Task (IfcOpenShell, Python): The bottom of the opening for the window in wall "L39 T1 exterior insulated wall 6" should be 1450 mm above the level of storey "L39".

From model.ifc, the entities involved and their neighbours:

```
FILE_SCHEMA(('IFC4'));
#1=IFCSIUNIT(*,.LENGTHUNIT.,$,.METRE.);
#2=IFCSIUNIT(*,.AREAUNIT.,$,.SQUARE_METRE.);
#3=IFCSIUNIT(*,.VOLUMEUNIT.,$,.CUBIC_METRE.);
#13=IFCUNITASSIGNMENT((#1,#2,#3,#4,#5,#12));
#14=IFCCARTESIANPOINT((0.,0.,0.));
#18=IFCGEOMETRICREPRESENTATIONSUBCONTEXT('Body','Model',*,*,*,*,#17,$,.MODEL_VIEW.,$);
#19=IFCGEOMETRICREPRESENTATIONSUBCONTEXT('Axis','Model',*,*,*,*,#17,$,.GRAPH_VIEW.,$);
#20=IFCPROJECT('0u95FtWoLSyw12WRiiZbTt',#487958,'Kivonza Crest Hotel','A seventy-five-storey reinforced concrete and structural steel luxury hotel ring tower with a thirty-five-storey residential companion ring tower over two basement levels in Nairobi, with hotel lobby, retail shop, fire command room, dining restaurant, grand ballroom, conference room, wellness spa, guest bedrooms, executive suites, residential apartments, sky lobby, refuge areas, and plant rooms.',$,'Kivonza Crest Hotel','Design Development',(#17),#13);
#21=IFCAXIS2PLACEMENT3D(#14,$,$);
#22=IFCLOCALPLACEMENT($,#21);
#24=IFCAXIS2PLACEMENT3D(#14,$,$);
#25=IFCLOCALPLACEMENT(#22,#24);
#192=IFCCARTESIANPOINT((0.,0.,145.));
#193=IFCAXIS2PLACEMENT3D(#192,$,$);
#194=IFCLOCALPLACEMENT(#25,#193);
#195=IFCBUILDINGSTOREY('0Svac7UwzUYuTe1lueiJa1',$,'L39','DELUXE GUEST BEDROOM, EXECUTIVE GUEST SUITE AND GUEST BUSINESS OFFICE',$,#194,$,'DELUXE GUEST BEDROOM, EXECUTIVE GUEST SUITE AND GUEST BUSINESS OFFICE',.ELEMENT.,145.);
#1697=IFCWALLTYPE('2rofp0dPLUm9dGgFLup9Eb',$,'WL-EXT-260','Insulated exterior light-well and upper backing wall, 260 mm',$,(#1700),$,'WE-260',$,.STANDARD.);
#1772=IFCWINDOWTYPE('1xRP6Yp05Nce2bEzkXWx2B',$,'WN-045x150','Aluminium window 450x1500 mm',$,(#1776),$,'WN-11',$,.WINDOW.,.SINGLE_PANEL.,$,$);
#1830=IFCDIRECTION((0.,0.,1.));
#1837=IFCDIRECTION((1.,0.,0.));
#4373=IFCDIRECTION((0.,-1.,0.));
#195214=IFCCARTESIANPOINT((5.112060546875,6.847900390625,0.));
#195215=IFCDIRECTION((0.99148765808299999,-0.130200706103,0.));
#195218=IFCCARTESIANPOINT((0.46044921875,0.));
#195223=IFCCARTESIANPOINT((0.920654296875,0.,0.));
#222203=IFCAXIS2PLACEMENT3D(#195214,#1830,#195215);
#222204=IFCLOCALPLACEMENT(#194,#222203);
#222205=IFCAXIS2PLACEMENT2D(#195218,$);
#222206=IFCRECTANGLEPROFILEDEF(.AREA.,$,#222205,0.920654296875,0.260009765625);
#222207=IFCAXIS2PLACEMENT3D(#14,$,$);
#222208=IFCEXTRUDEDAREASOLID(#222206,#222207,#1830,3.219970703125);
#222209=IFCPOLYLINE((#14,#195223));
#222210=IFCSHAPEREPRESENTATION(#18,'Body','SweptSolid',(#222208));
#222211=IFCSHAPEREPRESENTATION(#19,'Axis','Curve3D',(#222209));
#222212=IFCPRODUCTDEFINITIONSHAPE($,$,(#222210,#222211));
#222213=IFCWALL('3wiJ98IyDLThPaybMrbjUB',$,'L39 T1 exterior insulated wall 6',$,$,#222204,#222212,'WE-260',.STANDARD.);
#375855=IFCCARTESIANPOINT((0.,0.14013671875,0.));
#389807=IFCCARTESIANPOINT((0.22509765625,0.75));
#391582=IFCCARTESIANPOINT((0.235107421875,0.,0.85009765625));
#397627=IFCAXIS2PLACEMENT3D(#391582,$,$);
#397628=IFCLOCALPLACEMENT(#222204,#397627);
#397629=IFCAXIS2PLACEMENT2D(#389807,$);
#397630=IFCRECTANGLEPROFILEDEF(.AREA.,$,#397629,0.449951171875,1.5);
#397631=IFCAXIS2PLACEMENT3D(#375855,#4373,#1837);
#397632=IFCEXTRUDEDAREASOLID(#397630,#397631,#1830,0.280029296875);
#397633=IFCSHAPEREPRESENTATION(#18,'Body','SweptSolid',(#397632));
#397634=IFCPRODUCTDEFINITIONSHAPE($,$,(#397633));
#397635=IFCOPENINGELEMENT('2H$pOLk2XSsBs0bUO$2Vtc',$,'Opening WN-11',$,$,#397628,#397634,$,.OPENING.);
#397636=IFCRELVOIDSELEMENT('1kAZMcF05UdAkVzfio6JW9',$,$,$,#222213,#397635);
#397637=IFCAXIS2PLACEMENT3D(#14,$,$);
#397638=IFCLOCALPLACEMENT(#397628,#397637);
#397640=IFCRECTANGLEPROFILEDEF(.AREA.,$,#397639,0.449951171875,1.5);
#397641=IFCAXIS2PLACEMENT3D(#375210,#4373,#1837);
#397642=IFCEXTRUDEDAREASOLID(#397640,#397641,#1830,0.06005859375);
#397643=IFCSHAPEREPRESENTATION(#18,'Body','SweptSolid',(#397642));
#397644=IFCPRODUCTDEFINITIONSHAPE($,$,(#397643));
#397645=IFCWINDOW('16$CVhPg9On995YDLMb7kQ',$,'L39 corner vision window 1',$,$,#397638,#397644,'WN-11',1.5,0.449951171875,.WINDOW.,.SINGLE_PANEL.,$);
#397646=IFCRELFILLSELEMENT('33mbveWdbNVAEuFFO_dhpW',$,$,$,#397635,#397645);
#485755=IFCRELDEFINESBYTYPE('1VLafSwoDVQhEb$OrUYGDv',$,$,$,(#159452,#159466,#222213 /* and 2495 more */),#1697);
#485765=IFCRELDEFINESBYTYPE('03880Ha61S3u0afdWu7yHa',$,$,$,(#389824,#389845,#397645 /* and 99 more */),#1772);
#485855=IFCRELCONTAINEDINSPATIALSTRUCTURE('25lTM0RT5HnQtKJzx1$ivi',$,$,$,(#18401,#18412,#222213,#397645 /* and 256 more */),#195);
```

```python
import numpy as np
import ifcopenshell
import ifcopenshell.api.geometry
import ifcopenshell.geom
import ifcopenshell.util.element
import ifcopenshell.util.placement
import ifcopenshell.util.shape
import ifcopenshell.util.unit

model = ifcopenshell.open("model.ifc")
unit_scale = ifcopenshell.util.unit.calculate_unit_scale(model)

window = model.by_guid("16$CVhPg9On995YDLMb7kQ")
opening = window.FillsVoids[0].RelatingOpeningElement
storey = ifcopenshell.util.element.get_container(window, ifc_class="IfcBuildingStorey")
level = ifcopenshell.util.placement.get_local_placement(storey.ObjectPlacement)[2, 3]

# The opening's origin need not be at the sill, so measure its lowest point.
shape = ifcopenshell.geom.create_shape(ifcopenshell.geom.settings(), opening)
bottom = ifcopenshell.util.shape.get_shape_bottom_elevation(shape, shape.geometry) / unit_scale
dz = level + 1.45 / unit_scale - bottom

shift = np.array([0.0, 0.0, dz])
# The window is placed relative to its opening, so it follows when the opening moves.
matrix = ifcopenshell.util.placement.get_local_placement(opening.ObjectPlacement)
matrix[:3, 3] += shift
ifcopenshell.api.geometry.edit_object_placement(
    model, product=opening, matrix=matrix, is_si=False, should_transform_children=True
)

print(f"moved by {dz * unit_scale:+.3f} m")

model.write("model-out.ifc")
```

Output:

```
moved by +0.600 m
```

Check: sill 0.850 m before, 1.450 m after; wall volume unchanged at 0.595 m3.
